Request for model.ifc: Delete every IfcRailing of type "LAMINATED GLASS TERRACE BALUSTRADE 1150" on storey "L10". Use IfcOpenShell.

First a look at what the model holds.

```python
import ifcopenshell
import ifcopenshell.util.element

model = ifcopenshell.open("model.ifc")
print(model.schema)
storey = next(s for s in model.by_type("IfcBuildingStorey") if s.Name == "L10")
railings = [e for e in ifcopenshell.util.element.get_decomposition(storey) if e.is_a("IfcRailing")]
seen = {}
for e in railings:
    element_type = ifcopenshell.util.element.get_type(e)
    name = element_type.Name if element_type not in (None, e) else None
    seen[name] = seen.get(name, 0) + 1
for name, count in sorted(seen.items(), key=str):
    print(count, "x", name)
```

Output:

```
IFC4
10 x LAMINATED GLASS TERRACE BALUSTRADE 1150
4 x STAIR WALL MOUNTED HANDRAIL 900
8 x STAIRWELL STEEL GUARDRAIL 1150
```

```python
import ifcopenshell
import ifcopenshell.api.root
import ifcopenshell.util.element

model = ifcopenshell.open("model.ifc")

storey = next(s for s in model.by_type("IfcBuildingStorey") if s.Name == "L10")
railings = [e for e in ifcopenshell.util.element.get_decomposition(storey) if e.is_a("IfcRailing")]
targets = [e for e in railings if (t := ifcopenshell.util.element.get_type(e)) not in (None, e) and t.Name == "LAMINATED GLASS TERRACE BALUSTRADE 1150"]

for e in targets:
    ifcopenshell.api.root.remove_product(model, product=e)
print(len(targets), "removed")

model.write("model-out.ifc")
```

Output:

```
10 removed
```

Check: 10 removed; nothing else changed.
